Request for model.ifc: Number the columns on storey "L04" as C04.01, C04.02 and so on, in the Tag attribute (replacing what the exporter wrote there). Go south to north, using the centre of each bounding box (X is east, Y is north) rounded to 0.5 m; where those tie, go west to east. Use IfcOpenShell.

First a look at what the model holds.

```python
import ifcopenshell
import ifcopenshell.util.element
import ifcopenshell.util.placement

model = ifcopenshell.open("model.ifc")
print(model.schema)
storey = next(s for s in model.by_type("IfcBuildingStorey") if s.Name == "L04")
columns = [e for e in ifcopenshell.util.element.get_decomposition(storey) if e.is_a("IfcColumn")]
for e in sorted(columns, key=lambda e: e.id()):
    origin = ifcopenshell.util.placement.get_local_placement(e.ObjectPlacement)[:3, 3]
    print(e.id(), e.Tag, e.Name, origin.round(2) + 0.0, sep=" | ")
```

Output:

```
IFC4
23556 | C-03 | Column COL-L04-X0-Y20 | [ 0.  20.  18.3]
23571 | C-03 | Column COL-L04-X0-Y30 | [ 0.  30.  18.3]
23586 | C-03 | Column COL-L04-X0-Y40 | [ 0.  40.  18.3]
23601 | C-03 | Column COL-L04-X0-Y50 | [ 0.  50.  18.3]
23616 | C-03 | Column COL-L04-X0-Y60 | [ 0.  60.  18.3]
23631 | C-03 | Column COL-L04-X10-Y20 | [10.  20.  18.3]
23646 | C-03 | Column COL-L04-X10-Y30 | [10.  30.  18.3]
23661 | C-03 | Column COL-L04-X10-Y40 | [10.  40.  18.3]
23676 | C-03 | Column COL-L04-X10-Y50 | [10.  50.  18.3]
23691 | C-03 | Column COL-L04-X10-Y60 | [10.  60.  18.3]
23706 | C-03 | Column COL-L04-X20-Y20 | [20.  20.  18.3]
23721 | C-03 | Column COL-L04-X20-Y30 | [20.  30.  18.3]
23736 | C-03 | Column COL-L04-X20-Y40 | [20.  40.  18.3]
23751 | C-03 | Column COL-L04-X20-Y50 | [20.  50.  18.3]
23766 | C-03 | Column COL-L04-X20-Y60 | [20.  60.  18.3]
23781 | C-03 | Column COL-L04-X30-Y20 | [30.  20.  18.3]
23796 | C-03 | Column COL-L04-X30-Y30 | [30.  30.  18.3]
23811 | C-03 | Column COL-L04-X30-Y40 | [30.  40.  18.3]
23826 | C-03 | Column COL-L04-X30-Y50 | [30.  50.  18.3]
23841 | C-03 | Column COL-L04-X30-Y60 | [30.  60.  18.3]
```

```python
import ifcopenshell
import ifcopenshell.geom
import ifcopenshell.util.element
import ifcopenshell.util.shape

model = ifcopenshell.open("model.ifc")
settings = ifcopenshell.geom.settings()
settings.set("use-world-coords", True)


def centre(element):
    shape = ifcopenshell.geom.create_shape(settings, element)
    return ifcopenshell.util.shape.get_bbox_centroid(shape.geometry)


storey = next(s for s in model.by_type("IfcBuildingStorey") if s.Name == "L04")
columns = [e for e in ifcopenshell.util.element.get_decomposition(storey) if e.is_a("IfcColumn")]

# Insertion points can sit at a corner or the storey origin, so sort by the geometry (in metres).
centres = {e: centre(e) for e in columns}
columns.sort(key=lambda e: (round(centres[e][1] / 0.5), centres[e][0]))

for i, e in enumerate(columns, start=1):
    number = f"C04.{i:02d}"
    e.Tag = number
    print(e.id(), number)

model.write("model_edited.ifc")
```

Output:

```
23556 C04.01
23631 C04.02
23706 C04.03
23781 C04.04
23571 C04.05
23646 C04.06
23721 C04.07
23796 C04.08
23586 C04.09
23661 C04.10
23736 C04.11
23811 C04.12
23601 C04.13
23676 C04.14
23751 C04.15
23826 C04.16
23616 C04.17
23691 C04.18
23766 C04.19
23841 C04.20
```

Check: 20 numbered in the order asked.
